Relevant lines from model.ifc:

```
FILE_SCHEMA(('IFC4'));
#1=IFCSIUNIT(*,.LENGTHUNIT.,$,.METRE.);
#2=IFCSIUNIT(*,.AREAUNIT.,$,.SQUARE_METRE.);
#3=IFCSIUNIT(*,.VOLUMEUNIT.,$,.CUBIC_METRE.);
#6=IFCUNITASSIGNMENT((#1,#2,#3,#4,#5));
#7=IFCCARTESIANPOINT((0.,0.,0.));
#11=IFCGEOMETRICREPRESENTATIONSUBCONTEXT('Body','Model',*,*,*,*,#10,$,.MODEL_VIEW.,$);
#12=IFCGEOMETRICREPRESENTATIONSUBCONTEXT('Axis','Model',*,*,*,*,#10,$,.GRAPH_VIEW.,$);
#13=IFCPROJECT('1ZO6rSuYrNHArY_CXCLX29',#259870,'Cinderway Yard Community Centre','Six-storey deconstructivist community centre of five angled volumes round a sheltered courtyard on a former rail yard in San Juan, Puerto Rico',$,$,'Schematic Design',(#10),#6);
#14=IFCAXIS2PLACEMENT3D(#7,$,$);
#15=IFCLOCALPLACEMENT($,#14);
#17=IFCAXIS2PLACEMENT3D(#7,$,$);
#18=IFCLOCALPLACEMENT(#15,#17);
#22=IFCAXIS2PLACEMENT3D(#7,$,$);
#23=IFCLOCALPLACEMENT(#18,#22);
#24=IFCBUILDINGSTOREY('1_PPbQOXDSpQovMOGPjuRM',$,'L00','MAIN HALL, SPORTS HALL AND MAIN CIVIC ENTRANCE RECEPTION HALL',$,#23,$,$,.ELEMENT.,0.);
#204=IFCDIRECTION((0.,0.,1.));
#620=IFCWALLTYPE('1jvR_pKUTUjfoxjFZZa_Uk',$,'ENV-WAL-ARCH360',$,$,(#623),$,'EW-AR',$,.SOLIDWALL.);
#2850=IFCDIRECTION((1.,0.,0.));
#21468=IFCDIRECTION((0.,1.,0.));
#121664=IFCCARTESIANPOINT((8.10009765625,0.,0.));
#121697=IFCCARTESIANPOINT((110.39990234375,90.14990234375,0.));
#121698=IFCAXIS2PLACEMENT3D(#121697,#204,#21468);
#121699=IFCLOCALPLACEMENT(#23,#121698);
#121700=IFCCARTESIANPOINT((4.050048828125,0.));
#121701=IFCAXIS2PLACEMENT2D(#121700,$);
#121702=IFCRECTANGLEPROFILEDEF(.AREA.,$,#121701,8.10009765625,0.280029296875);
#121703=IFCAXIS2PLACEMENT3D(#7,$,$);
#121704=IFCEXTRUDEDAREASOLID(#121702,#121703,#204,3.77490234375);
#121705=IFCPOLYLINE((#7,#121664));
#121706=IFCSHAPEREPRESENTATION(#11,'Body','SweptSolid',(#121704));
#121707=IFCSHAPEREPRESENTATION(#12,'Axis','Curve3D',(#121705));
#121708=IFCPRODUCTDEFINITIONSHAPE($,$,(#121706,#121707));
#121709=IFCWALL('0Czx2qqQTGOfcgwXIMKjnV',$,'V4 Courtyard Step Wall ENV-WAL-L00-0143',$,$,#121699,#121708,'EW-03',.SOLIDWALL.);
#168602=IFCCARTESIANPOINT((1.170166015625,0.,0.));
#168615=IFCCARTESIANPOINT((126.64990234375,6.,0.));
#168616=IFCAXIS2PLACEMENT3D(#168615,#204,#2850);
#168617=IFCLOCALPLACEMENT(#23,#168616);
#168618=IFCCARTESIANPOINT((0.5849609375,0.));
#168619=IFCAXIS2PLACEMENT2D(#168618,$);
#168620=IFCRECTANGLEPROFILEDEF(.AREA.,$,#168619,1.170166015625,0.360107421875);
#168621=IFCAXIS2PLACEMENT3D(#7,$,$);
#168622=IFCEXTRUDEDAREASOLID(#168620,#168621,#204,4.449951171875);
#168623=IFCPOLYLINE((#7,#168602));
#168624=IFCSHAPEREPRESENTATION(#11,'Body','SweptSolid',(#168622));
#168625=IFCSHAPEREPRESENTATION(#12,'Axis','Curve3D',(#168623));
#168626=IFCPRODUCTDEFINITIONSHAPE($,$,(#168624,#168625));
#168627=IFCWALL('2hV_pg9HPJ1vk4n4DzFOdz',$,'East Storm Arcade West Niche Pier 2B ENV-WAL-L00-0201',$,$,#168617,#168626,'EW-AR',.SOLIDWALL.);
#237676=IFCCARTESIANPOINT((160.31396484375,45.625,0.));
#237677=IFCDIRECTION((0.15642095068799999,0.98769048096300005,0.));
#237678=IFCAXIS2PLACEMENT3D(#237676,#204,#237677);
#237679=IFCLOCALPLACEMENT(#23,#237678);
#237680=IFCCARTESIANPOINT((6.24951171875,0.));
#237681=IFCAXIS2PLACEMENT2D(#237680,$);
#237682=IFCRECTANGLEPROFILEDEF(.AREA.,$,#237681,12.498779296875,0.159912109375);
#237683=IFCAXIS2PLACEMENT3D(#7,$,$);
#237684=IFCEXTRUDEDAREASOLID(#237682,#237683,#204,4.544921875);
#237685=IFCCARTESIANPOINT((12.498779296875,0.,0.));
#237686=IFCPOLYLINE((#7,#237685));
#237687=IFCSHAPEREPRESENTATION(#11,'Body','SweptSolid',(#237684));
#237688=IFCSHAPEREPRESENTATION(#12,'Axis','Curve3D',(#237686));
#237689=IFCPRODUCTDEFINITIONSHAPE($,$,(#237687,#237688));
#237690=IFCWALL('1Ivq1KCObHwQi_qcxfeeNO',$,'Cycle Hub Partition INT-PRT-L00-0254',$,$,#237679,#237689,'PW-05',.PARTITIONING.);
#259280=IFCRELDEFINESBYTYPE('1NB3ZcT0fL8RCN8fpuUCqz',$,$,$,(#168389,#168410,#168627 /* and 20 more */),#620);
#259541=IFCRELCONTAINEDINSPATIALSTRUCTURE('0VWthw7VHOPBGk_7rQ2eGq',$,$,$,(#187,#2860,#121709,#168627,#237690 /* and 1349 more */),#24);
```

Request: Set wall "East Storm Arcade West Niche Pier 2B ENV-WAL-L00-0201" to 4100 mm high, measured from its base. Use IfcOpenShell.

```python
import ifcopenshell
import ifcopenshell.geom
import ifcopenshell.util.representation
import ifcopenshell.util.shape

model = ifcopenshell.open("model.ifc")
settings = ifcopenshell.geom.settings()


def volume(element):
    """Net volume in cubic metres, openings subtracted."""
    shape = ifcopenshell.geom.create_shape(settings, element)
    return ifcopenshell.util.shape.get_volume(shape.geometry)


wall = model.by_id(168627)
before = volume(wall)

body = ifcopenshell.util.representation.get_representation(wall, "Model", "Body")
solid = body.Items[0]
old_height = solid.Depth
solid.Depth = 4.1
after = volume(wall)

print(f"height {old_height:g} -> {solid.Depth:g}, volume {before:.3f} -> {after:.3f} m3")

model.write("model_rev.ifc")
```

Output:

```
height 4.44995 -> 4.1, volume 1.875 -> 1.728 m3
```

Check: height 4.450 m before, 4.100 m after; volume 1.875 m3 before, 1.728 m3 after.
